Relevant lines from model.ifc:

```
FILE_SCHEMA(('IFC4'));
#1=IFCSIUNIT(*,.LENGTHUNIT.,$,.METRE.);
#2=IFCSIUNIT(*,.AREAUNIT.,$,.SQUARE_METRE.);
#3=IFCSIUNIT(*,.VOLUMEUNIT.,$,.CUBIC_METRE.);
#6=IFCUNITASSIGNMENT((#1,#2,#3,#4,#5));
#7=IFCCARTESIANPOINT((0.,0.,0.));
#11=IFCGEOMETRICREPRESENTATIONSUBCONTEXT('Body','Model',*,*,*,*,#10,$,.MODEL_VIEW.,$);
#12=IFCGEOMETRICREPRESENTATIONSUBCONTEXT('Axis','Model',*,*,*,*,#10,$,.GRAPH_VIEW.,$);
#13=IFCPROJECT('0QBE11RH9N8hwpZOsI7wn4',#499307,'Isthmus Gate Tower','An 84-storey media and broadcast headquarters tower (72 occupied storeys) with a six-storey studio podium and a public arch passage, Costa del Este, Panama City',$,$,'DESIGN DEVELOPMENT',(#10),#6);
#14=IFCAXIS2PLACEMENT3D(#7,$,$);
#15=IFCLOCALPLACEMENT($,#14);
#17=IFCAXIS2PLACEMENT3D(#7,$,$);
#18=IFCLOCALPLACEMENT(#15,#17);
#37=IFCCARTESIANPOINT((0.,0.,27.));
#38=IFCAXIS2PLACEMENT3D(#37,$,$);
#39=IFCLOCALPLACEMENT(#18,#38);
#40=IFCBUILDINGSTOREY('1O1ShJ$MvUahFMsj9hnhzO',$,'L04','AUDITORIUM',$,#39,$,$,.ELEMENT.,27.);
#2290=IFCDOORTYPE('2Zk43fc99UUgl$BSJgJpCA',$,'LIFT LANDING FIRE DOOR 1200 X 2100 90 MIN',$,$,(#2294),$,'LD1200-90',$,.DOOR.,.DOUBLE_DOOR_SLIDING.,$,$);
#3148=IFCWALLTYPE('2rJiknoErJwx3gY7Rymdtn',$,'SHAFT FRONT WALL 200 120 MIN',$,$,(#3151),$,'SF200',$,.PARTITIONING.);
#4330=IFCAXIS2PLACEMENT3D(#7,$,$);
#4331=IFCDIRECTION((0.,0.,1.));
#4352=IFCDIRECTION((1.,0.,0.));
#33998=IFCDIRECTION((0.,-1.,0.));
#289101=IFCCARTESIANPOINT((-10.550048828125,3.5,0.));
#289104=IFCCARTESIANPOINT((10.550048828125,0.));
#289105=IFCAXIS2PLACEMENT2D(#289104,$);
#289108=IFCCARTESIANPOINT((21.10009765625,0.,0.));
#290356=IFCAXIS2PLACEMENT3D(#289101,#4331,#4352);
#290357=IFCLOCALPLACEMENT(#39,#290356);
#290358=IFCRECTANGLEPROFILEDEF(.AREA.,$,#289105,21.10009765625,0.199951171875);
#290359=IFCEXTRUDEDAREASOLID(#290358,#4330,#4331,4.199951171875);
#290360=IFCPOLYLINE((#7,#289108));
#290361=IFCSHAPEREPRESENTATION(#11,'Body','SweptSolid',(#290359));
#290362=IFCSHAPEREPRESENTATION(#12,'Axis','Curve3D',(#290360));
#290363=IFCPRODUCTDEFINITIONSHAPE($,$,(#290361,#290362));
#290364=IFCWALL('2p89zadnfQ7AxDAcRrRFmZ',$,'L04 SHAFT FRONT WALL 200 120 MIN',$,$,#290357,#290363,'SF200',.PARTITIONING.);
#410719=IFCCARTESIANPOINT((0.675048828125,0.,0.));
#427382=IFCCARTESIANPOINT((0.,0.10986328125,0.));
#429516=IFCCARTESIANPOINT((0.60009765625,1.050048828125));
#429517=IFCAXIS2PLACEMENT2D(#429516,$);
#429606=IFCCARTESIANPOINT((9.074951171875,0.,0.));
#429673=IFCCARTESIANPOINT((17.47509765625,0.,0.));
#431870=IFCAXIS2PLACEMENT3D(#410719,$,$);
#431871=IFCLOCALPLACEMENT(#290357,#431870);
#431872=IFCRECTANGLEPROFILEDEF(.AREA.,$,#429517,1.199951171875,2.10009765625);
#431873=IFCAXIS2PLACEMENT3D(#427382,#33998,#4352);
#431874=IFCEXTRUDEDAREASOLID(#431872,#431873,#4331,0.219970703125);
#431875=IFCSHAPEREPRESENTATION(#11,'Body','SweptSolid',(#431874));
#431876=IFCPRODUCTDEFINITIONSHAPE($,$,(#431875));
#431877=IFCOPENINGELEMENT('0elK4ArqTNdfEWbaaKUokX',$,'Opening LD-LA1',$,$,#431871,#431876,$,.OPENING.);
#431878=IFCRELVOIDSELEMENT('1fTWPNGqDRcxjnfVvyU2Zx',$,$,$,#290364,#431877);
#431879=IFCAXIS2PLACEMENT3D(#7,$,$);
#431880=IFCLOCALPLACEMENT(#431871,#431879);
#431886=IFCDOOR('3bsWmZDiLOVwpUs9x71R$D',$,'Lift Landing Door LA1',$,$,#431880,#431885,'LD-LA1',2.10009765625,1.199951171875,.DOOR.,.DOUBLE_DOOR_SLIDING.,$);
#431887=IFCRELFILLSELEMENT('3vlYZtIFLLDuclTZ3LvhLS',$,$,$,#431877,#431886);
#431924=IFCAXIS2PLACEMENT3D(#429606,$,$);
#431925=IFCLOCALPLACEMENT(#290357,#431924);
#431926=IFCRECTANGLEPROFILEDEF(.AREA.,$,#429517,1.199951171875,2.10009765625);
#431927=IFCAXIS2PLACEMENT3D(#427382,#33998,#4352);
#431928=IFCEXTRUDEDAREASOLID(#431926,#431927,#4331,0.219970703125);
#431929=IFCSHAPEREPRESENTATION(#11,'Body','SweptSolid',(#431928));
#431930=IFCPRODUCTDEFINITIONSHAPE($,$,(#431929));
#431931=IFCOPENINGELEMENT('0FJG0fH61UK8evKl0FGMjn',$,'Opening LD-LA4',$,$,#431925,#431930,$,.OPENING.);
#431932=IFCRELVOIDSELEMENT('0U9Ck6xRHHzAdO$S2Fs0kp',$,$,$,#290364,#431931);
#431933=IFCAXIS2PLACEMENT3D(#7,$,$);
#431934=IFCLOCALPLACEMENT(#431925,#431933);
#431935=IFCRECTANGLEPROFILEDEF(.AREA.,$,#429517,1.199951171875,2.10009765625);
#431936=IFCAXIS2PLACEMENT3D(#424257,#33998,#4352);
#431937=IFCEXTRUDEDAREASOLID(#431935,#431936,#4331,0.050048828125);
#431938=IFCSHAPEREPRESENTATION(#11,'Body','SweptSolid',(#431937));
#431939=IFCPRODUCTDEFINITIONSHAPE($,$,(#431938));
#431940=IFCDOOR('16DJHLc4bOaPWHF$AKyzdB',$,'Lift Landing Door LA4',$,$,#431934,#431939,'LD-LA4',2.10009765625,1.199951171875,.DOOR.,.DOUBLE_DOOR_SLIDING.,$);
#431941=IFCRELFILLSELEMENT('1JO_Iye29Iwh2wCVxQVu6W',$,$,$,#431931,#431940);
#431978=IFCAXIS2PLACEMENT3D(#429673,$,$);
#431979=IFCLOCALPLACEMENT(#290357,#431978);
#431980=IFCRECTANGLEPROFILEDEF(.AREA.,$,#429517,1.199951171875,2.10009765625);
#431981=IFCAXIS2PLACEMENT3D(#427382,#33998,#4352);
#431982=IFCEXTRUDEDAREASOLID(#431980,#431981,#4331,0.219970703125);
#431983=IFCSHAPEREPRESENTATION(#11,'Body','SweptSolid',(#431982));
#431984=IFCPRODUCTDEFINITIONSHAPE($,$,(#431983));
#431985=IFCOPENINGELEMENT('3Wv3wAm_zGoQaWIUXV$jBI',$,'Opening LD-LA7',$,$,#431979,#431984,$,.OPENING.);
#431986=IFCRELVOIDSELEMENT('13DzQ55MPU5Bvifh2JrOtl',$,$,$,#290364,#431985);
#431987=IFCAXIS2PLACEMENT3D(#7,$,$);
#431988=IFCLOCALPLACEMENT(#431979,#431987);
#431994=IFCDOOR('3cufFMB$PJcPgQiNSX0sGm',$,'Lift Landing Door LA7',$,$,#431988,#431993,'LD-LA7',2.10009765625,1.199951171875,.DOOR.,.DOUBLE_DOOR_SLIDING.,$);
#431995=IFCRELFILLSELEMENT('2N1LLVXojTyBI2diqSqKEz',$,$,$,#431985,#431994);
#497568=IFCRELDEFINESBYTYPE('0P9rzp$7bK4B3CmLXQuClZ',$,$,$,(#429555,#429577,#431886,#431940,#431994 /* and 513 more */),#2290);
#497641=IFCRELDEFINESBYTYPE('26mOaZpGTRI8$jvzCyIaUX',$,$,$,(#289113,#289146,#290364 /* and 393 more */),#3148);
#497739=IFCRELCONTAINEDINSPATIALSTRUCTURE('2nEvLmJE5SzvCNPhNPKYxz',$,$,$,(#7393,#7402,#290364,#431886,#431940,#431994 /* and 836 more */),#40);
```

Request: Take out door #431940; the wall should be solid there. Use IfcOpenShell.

```python
import ifcopenshell
import ifcopenshell.api.feature
import ifcopenshell.api.root
import ifcopenshell.geom
import ifcopenshell.util.shape

model = ifcopenshell.open("model.ifc")
settings = ifcopenshell.geom.settings()


def volume(element):
    """Net volume in cubic metres, openings subtracted."""
    shape = ifcopenshell.geom.create_shape(settings, element)
    return ifcopenshell.util.shape.get_volume(shape.geometry)


door = model.by_id(431940)
opening = door.FillsVoids[0].RelatingOpeningElement
wall = opening.VoidsElements[0].RelatingBuildingElement
before = volume(wall)

ifcopenshell.api.root.remove_product(model, product=door)
ifcopenshell.api.feature.remove_feature(model, feature=opening)

after = volume(wall)

print(f"wall volume {before:.3f} -> {after:.3f} m3")

model.write("model_v2.ifc")
```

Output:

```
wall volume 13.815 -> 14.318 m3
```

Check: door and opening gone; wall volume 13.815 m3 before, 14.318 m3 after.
